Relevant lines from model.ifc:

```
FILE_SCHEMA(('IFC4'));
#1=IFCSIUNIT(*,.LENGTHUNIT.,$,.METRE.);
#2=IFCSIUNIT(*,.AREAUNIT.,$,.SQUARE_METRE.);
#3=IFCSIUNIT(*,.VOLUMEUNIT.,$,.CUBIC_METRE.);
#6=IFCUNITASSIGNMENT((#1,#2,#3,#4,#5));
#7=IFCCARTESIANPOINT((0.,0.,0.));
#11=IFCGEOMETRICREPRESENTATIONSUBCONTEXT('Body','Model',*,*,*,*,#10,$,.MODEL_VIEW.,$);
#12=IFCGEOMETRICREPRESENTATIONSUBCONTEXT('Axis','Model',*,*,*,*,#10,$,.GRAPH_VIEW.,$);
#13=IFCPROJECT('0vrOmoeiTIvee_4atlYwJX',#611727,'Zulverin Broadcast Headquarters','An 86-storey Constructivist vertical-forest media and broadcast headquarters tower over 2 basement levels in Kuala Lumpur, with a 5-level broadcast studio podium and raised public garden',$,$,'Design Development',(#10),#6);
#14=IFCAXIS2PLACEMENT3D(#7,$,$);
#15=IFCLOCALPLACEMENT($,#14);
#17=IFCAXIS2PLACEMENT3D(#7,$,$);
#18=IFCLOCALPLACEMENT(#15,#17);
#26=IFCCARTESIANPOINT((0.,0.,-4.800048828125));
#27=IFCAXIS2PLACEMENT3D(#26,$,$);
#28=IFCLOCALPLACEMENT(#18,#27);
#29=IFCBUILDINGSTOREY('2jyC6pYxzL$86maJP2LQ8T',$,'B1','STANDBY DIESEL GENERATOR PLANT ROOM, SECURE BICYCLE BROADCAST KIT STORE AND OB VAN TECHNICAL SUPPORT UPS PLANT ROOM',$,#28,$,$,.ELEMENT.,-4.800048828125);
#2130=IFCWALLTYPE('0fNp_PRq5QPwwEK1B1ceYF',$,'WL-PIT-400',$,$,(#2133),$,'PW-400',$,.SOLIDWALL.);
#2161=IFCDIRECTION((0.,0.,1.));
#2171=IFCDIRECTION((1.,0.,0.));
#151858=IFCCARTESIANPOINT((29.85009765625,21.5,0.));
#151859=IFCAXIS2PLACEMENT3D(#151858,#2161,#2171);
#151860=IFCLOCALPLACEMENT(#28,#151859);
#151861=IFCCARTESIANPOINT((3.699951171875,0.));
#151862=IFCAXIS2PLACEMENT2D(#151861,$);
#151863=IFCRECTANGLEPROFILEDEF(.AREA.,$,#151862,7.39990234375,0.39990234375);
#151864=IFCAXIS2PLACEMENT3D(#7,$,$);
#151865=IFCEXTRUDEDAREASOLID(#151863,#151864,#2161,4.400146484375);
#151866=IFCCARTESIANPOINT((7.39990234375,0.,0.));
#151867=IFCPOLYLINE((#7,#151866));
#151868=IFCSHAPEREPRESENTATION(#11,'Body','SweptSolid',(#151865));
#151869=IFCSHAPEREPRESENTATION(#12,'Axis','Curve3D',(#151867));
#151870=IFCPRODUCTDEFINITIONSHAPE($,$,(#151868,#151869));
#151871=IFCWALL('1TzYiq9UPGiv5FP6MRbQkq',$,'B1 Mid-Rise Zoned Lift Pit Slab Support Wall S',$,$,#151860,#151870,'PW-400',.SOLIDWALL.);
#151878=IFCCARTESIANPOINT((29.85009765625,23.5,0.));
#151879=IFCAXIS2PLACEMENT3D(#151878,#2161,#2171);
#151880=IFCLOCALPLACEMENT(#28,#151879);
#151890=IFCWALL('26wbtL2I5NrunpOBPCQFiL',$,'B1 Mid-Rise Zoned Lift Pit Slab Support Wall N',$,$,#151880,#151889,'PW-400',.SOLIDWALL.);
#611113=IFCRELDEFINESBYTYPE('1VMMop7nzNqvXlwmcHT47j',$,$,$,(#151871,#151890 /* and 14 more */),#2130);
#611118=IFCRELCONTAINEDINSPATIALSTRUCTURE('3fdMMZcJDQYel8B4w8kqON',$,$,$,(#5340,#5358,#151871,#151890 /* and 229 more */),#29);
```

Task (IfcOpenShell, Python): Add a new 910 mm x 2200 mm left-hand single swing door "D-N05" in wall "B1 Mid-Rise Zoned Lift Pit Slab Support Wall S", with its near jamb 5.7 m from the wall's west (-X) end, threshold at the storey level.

```python
import numpy as np
import ifcopenshell
import ifcopenshell.api.feature
import ifcopenshell.api.geometry
import ifcopenshell.api.root
import ifcopenshell.api.spatial
import ifcopenshell.geom
import ifcopenshell.util.element
import ifcopenshell.util.placement
import ifcopenshell.util.representation
import ifcopenshell.util.shape
import ifcopenshell.util.unit

model = ifcopenshell.open("model.ifc")
unit_scale = ifcopenshell.util.unit.calculate_unit_scale(model)
settings = ifcopenshell.geom.settings()


def volume(element):
    """Net volume in cubic metres, openings subtracted."""
    shape = ifcopenshell.geom.create_shape(settings, element)
    return ifcopenshell.util.shape.get_volume(shape.geometry)


wall = model.by_guid("1TzYiq9UPGiv5FP6MRbQkq")
storey = ifcopenshell.util.element.get_container(wall, ifc_class="IfcBuildingStorey")
context = ifcopenshell.util.representation.get_context(model, "Model", "Body", "MODEL_VIEW")
before = volume(wall)

width, height, from_end, sill = 0.91, 2.2, 5.7, 0.0  # metres

# The wall runs along its own X axis, and the end named is its -X end.
wall_shape = ifcopenshell.geom.create_shape(settings, wall)
x, y, z = ifcopenshell.util.shape.get_vertices(wall_shape.geometry).T
start = x.min() + from_end
face, thickness = float(y.min()), float(y.max() - y.min())
wall_matrix = ifcopenshell.util.placement.get_local_placement(wall.ObjectPlacement)
level = ifcopenshell.util.placement.get_local_placement(storey.ObjectPlacement)[2, 3]


def in_wall(x, y):
    """Placement at x, y metres in the wall's axes, at sill height."""
    matrix = wall_matrix.copy()
    matrix[:, 3] = wall_matrix @ np.array([x / unit_scale, y / unit_scale, 0.0, 1.0])
    matrix[2, 3] = level + sill / unit_scale
    return matrix


# Opening: a box that overshoots both wall faces by 50 mm.
opening = ifcopenshell.api.root.create_entity(model, ifc_class="IfcOpeningElement", predefined_type="OPENING")
box = ifcopenshell.api.geometry.add_wall_representation(
    model, context=context, length=width, height=height, thickness=thickness + 0.1
)
ifcopenshell.api.geometry.assign_representation(model, product=opening, representation=box)
ifcopenshell.api.geometry.edit_object_placement(model, product=opening, matrix=in_wall(start, face - 0.05), is_si=False)
ifcopenshell.api.feature.add_feature(model, feature=opening, element=wall)

door = ifcopenshell.api.root.create_entity(model, ifc_class="IfcDoor", name="D-N05", predefined_type="DOOR")
door.OverallWidth, door.OverallHeight = width / unit_scale, height / unit_scale
door.OperationType = "SINGLE_SWING_LEFT"
body = ifcopenshell.api.geometry.add_door_representation(
    model,
    context=context,
    overall_width=door.OverallWidth,
    overall_height=door.OverallHeight,
    operation_type="SINGLE_SWING_LEFT",
    lining_properties={"LiningDepth": thickness / unit_scale, "ThresholdDepth": thickness / unit_scale},
)
ifcopenshell.api.geometry.assign_representation(model, product=door, representation=body)
ifcopenshell.api.spatial.assign_container(model, products=[door], relating_structure=storey)
ifcopenshell.api.feature.add_filling(model, opening=opening, element=door)

# The lining spans the wall, so the door starts at the wall face.
ifcopenshell.api.geometry.edit_object_placement(model, product=door, matrix=in_wall(start, face), is_si=False)

after = volume(wall)

print(f"wall volume {before:.3f} -> {after:.3f} m3")

model.write("model-out.ifc")
```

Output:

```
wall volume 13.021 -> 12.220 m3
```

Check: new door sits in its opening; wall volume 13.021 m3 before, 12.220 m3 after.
